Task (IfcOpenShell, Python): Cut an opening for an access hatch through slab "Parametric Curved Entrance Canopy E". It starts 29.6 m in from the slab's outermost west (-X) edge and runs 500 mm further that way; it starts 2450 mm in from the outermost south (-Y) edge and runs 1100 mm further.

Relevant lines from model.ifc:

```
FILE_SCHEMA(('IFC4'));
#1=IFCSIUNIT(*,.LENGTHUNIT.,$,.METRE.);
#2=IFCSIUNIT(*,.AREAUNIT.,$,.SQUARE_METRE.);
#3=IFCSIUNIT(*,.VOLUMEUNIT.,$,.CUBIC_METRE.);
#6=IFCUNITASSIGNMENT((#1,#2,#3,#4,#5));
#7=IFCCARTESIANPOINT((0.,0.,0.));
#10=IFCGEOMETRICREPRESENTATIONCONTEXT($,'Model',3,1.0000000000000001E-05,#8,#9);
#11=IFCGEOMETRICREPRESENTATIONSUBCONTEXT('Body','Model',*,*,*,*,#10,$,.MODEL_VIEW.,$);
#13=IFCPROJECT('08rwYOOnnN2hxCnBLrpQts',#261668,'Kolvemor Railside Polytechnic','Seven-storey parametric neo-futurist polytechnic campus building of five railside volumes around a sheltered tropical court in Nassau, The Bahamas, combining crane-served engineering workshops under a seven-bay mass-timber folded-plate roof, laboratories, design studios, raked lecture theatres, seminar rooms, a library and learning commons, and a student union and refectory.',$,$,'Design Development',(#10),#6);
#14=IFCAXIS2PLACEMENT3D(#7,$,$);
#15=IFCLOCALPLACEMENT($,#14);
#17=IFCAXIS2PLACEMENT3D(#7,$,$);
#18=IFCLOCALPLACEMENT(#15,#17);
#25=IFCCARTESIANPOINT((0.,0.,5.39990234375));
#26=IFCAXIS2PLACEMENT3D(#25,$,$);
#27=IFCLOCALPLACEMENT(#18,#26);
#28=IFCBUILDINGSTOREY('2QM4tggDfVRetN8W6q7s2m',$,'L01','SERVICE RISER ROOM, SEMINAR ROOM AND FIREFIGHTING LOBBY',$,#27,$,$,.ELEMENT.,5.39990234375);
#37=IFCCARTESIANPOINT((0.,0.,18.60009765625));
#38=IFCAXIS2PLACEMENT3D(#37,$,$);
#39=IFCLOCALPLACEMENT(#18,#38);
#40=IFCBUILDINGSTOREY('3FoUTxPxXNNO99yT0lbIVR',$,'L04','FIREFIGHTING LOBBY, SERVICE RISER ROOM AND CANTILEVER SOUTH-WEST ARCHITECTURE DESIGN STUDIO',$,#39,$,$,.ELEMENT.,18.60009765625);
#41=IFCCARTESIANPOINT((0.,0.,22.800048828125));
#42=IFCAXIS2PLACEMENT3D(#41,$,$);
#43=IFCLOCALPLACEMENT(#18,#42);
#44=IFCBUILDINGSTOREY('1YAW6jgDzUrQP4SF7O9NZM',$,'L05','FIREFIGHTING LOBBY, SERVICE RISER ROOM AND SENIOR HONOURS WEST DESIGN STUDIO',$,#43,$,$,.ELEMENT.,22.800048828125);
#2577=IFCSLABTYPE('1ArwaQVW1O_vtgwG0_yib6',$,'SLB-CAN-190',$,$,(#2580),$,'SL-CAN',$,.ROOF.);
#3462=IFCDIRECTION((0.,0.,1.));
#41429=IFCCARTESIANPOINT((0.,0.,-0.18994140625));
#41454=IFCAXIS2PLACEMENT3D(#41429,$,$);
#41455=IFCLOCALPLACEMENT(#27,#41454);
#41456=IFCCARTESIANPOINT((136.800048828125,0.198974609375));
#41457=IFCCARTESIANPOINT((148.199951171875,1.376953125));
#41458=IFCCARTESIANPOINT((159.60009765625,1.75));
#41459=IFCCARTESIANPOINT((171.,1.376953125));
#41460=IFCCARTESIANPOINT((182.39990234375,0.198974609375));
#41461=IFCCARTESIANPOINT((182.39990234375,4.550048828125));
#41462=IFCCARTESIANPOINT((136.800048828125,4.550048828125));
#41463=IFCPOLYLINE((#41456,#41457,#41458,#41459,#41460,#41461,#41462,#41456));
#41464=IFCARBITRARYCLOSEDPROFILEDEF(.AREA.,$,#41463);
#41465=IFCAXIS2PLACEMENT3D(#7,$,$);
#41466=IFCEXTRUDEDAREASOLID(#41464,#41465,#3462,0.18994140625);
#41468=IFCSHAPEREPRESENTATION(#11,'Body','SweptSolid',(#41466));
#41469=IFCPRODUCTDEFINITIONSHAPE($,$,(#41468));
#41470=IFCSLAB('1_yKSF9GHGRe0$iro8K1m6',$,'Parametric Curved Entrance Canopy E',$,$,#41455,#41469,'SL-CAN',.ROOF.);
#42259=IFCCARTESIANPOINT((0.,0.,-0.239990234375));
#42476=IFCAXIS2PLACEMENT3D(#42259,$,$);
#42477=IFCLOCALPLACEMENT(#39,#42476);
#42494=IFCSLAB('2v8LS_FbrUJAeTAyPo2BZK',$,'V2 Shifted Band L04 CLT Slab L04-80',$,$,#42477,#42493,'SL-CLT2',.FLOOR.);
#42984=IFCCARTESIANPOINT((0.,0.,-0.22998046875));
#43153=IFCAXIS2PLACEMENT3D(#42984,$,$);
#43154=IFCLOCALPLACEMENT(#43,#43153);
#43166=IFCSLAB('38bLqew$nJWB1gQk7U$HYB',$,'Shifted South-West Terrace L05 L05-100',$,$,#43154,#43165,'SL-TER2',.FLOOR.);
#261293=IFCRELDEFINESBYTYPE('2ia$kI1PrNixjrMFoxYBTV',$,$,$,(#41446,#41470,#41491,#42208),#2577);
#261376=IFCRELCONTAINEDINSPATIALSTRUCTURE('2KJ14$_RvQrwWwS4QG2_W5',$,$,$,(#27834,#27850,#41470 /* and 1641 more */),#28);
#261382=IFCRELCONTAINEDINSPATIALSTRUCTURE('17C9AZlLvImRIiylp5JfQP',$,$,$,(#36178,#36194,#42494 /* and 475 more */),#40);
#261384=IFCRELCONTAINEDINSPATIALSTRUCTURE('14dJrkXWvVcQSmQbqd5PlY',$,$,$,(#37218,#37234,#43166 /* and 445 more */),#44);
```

```python
import numpy as np
import ifcopenshell
import ifcopenshell.api.feature
import ifcopenshell.api.geometry
import ifcopenshell.api.root
import ifcopenshell.geom
import ifcopenshell.util.placement
import ifcopenshell.util.representation
import ifcopenshell.util.shape
import ifcopenshell.util.unit

model = ifcopenshell.open("model.ifc")
unit_scale = ifcopenshell.util.unit.calculate_unit_scale(model)
settings = ifcopenshell.geom.settings()


def volume(element):
    """Net volume in cubic metres, openings subtracted."""
    shape = ifcopenshell.geom.create_shape(settings, element)
    return ifcopenshell.util.shape.get_volume(shape.geometry)


slab = model.by_id(41470)
before = volume(slab)

# Extent in the slab's own axes, in metres. The edges named are its -X and -Y sides.
slab_shape = ifcopenshell.geom.create_shape(settings, slab)
vertices = ifcopenshell.util.shape.get_vertices(slab_shape.geometry)
x_min, y_min, bottom = vertices.min(axis=0)
top = vertices[:, 2].max()

opening = ifcopenshell.api.root.create_entity(model, ifc_class="IfcOpeningElement", name="Access hatch opening", predefined_type="OPENING")
context = ifcopenshell.util.representation.get_context(model, "Model", "Body", "MODEL_VIEW")
width, depth = 0.5, 1.1
outline = [(0.0, 0.0), (width, 0.0), (width, depth), (0.0, depth), (0.0, 0.0)]
# Overshoot both faces by 50 mm so the cut is clean.
shape = ifcopenshell.api.geometry.add_slab_representation(
    model, context=context, depth=top - bottom + 0.1, polyline=outline
)
ifcopenshell.api.geometry.assign_representation(model, product=opening, representation=shape)

matrix = ifcopenshell.util.placement.get_local_placement(slab.ObjectPlacement)
matrix[:, 3] = matrix @ np.append(np.array([x_min + 29.6, y_min + 2.45, bottom - 0.05]) / unit_scale, 1.0)
ifcopenshell.api.geometry.edit_object_placement(model, product=opening, matrix=matrix, is_si=False)
ifcopenshell.api.feature.add_feature(model, feature=opening, element=slab)

after = volume(slab)

print(f"slab volume {before:.3f} -> {after:.3f} m3")

model.write("model_edited.ifc")
```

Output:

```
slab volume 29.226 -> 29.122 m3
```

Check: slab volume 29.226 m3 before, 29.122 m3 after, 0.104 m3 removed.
